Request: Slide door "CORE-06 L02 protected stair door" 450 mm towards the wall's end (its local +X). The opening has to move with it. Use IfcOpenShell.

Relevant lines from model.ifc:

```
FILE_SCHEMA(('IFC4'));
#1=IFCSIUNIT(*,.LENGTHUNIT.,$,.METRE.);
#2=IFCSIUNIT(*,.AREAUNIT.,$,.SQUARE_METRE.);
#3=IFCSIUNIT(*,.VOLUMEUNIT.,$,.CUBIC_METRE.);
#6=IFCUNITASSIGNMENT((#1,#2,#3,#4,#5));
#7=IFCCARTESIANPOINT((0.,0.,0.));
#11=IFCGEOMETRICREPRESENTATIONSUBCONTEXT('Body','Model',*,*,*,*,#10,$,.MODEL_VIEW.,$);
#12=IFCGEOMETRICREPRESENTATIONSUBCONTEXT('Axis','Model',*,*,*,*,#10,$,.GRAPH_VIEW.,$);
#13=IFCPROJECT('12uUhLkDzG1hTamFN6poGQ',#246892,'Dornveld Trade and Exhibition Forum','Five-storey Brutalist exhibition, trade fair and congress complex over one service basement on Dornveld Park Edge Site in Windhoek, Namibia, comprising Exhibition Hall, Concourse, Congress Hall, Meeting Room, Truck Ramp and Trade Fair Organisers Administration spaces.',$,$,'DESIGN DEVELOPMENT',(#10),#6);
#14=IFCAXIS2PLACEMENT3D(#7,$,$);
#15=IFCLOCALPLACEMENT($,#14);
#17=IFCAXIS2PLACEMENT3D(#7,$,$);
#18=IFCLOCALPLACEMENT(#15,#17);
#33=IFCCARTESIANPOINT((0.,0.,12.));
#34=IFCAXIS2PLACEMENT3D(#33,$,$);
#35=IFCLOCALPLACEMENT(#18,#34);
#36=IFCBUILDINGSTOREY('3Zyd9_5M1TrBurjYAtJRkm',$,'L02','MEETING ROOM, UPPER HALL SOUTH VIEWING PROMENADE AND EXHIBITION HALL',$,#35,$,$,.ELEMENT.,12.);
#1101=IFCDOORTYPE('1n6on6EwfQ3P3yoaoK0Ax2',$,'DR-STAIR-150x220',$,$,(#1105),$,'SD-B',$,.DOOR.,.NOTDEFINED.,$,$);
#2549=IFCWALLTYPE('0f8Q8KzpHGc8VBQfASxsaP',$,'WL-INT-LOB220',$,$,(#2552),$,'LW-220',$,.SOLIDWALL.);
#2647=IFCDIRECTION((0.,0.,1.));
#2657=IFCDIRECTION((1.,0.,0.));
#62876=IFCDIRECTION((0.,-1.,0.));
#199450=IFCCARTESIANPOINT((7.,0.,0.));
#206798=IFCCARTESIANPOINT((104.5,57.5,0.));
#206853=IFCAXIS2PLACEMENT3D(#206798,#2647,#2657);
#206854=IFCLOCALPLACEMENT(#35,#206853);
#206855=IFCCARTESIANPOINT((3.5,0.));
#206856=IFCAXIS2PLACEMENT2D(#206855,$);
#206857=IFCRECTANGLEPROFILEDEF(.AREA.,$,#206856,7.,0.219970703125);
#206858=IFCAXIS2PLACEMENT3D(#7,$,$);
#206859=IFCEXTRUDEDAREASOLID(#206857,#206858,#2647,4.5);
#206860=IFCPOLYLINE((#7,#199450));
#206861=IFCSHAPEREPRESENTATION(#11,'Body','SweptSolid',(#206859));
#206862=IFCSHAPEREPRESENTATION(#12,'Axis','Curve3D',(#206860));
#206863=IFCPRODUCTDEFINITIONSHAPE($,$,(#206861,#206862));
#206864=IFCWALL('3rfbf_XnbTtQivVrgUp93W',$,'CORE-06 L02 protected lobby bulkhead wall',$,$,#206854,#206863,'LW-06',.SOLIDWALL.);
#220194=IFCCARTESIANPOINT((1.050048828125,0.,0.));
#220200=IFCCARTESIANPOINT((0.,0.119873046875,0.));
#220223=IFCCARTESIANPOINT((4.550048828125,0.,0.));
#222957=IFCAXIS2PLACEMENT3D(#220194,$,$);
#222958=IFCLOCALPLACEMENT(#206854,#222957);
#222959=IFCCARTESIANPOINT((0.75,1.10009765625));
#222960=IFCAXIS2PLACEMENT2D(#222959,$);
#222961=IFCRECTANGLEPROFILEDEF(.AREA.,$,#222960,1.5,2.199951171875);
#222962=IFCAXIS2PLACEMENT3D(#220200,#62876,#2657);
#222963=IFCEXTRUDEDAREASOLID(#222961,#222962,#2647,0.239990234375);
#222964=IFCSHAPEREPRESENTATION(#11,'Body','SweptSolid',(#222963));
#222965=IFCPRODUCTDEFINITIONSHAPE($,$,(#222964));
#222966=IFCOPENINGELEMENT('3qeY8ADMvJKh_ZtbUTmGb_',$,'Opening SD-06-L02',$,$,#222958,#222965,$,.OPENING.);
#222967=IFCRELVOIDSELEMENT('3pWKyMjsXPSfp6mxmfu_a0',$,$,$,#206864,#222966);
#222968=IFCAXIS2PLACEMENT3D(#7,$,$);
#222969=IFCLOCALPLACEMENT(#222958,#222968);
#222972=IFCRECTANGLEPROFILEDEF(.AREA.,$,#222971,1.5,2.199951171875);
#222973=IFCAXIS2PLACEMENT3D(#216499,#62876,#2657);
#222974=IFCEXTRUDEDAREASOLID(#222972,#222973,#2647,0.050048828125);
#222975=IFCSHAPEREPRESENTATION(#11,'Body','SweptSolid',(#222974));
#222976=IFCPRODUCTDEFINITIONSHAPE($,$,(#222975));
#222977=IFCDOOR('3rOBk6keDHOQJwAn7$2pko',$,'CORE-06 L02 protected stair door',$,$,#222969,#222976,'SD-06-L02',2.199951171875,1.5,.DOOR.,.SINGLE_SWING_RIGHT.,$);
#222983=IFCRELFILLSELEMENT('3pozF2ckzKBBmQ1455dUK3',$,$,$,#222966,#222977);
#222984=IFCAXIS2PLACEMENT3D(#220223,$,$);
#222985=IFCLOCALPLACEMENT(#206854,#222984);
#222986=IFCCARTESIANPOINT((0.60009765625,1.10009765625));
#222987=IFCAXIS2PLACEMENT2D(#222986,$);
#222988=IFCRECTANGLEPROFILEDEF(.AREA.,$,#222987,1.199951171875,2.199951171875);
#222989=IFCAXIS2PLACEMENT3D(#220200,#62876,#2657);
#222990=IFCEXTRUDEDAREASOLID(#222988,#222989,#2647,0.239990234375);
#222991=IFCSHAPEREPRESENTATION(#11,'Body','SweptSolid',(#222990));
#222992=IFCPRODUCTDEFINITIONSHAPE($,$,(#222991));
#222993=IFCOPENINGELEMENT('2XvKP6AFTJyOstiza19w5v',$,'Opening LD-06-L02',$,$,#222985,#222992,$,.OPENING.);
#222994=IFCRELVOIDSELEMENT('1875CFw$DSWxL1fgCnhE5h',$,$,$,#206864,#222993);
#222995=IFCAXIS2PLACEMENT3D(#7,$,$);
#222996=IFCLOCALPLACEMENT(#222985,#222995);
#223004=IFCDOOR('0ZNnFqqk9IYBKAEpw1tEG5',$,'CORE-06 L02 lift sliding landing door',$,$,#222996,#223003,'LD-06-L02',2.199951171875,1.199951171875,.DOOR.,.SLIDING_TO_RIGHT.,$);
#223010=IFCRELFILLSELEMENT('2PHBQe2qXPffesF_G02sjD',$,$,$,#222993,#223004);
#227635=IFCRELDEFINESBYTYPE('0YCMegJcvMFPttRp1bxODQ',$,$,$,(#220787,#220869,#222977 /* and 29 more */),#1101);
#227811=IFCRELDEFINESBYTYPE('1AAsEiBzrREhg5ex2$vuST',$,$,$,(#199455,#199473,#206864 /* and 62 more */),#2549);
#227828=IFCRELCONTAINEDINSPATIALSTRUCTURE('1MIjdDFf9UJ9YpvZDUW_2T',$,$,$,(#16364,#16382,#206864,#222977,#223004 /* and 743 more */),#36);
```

```python
import ifcopenshell
import ifcopenshell.api.geometry
import ifcopenshell.util.placement
import ifcopenshell.util.unit

model = ifcopenshell.open("model.ifc")
unit_scale = ifcopenshell.util.unit.calculate_unit_scale(model)

door = model.by_id(222977)
opening = door.FillsVoids[0].RelatingOpeningElement
wall = opening.VoidsElements[0].RelatingBuildingElement

wall_matrix = ifcopenshell.util.placement.get_local_placement(wall.ObjectPlacement)
shift = wall_matrix[:3, 0] * 0.45 / unit_scale
before = ifcopenshell.util.placement.get_local_placement(door.ObjectPlacement)[:3, 3].copy()

# The door is placed relative to its opening, so it follows when the opening moves.
matrix = ifcopenshell.util.placement.get_local_placement(opening.ObjectPlacement)
matrix[:3, 3] += shift
ifcopenshell.api.geometry.edit_object_placement(
    model, product=opening, matrix=matrix, is_si=False, should_transform_children=True
)

after = ifcopenshell.util.placement.get_local_placement(door.ObjectPlacement)[:3, 3]
print("door moved by", (after - before).round(3) + 0.0)

model.write("model_edited.ifc")
```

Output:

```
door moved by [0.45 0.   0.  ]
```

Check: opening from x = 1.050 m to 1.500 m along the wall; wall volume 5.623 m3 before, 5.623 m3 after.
